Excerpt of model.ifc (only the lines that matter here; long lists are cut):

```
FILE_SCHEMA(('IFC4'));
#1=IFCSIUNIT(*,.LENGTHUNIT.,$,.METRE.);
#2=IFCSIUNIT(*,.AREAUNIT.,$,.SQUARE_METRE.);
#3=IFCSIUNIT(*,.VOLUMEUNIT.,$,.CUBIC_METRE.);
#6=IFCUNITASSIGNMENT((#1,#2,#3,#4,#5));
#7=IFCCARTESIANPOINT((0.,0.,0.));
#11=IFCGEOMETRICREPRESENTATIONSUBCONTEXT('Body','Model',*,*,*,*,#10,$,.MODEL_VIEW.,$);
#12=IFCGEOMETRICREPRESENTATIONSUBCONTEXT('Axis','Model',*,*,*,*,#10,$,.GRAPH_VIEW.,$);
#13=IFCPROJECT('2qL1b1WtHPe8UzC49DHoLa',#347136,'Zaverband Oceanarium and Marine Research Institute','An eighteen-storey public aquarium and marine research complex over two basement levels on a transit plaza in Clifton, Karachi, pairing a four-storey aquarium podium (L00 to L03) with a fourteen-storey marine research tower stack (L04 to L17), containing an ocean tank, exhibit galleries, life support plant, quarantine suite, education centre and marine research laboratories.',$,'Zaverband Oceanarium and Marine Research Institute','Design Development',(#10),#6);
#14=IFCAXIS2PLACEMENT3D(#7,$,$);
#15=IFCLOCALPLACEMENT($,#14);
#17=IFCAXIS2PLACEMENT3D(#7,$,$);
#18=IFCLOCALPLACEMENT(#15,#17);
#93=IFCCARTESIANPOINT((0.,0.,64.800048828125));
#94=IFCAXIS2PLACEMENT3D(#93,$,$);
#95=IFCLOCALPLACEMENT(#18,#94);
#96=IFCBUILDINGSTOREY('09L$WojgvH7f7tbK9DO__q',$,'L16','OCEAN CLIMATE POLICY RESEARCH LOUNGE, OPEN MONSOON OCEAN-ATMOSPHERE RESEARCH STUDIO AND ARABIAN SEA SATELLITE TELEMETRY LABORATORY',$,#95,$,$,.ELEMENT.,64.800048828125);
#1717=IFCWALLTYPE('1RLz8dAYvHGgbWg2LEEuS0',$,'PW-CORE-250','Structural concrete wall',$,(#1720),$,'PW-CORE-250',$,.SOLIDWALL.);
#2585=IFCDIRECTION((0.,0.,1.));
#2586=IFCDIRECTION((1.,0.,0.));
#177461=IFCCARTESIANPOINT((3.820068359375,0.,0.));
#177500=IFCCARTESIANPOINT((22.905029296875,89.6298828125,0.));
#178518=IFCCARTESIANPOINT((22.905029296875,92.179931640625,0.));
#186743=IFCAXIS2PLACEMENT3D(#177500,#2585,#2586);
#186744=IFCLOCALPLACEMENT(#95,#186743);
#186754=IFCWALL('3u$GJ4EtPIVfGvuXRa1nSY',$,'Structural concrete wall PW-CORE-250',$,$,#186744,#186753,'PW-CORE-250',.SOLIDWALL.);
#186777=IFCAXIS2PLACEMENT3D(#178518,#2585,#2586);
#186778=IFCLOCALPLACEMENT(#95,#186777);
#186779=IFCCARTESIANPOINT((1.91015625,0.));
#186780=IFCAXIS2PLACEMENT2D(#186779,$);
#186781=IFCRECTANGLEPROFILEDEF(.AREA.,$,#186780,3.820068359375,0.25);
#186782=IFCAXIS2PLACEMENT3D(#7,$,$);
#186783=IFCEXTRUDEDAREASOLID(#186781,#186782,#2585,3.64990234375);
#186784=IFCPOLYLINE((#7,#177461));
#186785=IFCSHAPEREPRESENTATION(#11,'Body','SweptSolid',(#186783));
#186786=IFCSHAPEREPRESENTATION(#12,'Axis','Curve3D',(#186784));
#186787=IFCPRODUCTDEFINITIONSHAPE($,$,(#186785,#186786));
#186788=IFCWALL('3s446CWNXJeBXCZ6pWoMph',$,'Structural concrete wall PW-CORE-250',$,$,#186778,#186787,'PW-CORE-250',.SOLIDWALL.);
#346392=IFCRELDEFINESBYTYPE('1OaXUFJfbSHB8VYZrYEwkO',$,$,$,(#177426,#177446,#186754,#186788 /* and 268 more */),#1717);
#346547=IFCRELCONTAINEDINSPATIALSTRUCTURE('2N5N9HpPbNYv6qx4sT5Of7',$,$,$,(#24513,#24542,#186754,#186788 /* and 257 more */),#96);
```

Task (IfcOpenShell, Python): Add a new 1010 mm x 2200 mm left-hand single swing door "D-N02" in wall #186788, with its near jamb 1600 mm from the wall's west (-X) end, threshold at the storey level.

```python
import numpy as np
import ifcopenshell
import ifcopenshell.api.feature
import ifcopenshell.api.geometry
import ifcopenshell.api.root
import ifcopenshell.api.spatial
import ifcopenshell.geom
import ifcopenshell.util.element
import ifcopenshell.util.placement
import ifcopenshell.util.representation
import ifcopenshell.util.shape
import ifcopenshell.util.unit

model = ifcopenshell.open("model.ifc")
unit_scale = ifcopenshell.util.unit.calculate_unit_scale(model)
settings = ifcopenshell.geom.settings()


def volume(element):
    """Net volume in cubic metres, openings subtracted."""
    shape = ifcopenshell.geom.create_shape(settings, element)
    return ifcopenshell.util.shape.get_volume(shape.geometry)


wall = model.by_guid("3s446CWNXJeBXCZ6pWoMph")
storey = ifcopenshell.util.element.get_container(wall, ifc_class="IfcBuildingStorey")
context = ifcopenshell.util.representation.get_context(model, "Model", "Body", "MODEL_VIEW")
before = volume(wall)

width, height, from_end, sill = 1.01, 2.2, 1.6, 0.0  # metres

# The wall runs along its own X axis, and the end named is its -X end.
wall_shape = ifcopenshell.geom.create_shape(settings, wall)
x, y, z = ifcopenshell.util.shape.get_vertices(wall_shape.geometry).T
start = x.min() + from_end
face, thickness = float(y.min()), float(y.max() - y.min())
wall_matrix = ifcopenshell.util.placement.get_local_placement(wall.ObjectPlacement)
level = ifcopenshell.util.placement.get_local_placement(storey.ObjectPlacement)[2, 3]


def in_wall(x, y):
    """Placement at x, y metres in the wall's axes, at sill height."""
    matrix = wall_matrix.copy()
    matrix[:, 3] = wall_matrix @ np.array([x / unit_scale, y / unit_scale, 0.0, 1.0])
    matrix[2, 3] = level + sill / unit_scale
    return matrix


# Opening: a box that overshoots both wall faces by 50 mm.
opening = ifcopenshell.api.root.create_entity(model, ifc_class="IfcOpeningElement", predefined_type="OPENING")
box = ifcopenshell.api.geometry.add_wall_representation(
    model, context=context, length=width, height=height, thickness=thickness + 0.1
)
ifcopenshell.api.geometry.assign_representation(model, product=opening, representation=box)
ifcopenshell.api.geometry.edit_object_placement(model, product=opening, matrix=in_wall(start, face - 0.05), is_si=False)
ifcopenshell.api.feature.add_feature(model, feature=opening, element=wall)

door = ifcopenshell.api.root.create_entity(model, ifc_class="IfcDoor", name="D-N02", predefined_type="DOOR")
door.OverallWidth, door.OverallHeight = width / unit_scale, height / unit_scale
door.OperationType = "SINGLE_SWING_LEFT"
body = ifcopenshell.api.geometry.add_door_representation(
    model,
    context=context,
    overall_width=door.OverallWidth,
    overall_height=door.OverallHeight,
    operation_type="SINGLE_SWING_LEFT",
    lining_properties={"LiningDepth": thickness / unit_scale, "ThresholdDepth": thickness / unit_scale},
)
ifcopenshell.api.geometry.assign_representation(model, product=door, representation=body)
ifcopenshell.api.spatial.assign_container(model, products=[door], relating_structure=storey)
ifcopenshell.api.feature.add_filling(model, opening=opening, element=door)

# The lining spans the wall, so the door starts at the wall face.
ifcopenshell.api.geometry.edit_object_placement(model, product=door, matrix=in_wall(start, face), is_si=False)

after = volume(wall)

print(f"wall volume {before:.3f} -> {after:.3f} m3")

model.write("model_rev.ifc")
```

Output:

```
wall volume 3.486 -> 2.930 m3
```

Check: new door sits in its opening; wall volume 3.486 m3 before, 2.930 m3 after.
